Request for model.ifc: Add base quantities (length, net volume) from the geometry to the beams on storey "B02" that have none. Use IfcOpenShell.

First a look at what the model holds.

```python
import ifcopenshell
import ifcopenshell.util.element
import ifcopenshell.util.unit

model = ifcopenshell.open("model.ifc")
print(model.schema)
for unit_type in ("LENGTHUNIT", "AREAUNIT", "VOLUMEUNIT"):
    print(unit_type, ifcopenshell.util.unit.calculate_unit_scale(model, unit_type))
storey = next(s for s in model.by_type("IfcBuildingStorey") if s.Name == "B02")
beams = [e for e in ifcopenshell.util.element.get_decomposition(storey) if e.is_a("IfcBeam")]
for e in sorted(beams, key=lambda e: e.id()):
    print(e.id(), e.is_a(), e.Name, list(ifcopenshell.util.element.get_psets(e, qtos_only=True)), sep=" | ")
```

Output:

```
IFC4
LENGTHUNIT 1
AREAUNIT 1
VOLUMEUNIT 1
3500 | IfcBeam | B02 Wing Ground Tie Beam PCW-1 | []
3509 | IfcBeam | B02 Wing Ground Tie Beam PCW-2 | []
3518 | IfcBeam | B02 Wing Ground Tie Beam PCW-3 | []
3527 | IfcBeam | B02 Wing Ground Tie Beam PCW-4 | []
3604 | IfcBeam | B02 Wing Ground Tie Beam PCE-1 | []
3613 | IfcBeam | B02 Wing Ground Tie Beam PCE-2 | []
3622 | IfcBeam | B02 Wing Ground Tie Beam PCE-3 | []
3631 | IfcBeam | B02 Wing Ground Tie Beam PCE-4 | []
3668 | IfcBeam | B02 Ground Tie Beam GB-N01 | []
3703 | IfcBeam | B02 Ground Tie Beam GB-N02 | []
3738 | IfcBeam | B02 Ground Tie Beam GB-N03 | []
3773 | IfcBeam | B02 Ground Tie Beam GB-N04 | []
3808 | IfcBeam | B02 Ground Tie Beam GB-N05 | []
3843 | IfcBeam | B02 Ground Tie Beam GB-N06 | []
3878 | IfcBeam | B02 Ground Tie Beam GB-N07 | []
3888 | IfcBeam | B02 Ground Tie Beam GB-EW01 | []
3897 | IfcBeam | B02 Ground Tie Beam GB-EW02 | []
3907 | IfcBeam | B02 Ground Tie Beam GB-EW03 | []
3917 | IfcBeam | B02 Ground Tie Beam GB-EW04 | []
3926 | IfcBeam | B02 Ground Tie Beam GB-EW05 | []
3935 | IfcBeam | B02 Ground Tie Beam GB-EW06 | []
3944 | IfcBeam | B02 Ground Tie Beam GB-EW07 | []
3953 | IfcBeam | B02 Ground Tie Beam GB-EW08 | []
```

```python
import ifcopenshell
import ifcopenshell.api.pset
import ifcopenshell.geom
import ifcopenshell.util.element
import ifcopenshell.util.shape
import ifcopenshell.util.unit

model = ifcopenshell.open("model.ifc")
unit_scale = ifcopenshell.util.unit.calculate_unit_scale(model)
volume_scale = ifcopenshell.util.unit.calculate_unit_scale(model, "VOLUMEUNIT")
settings = ifcopenshell.geom.settings()

storey = next(s for s in model.by_type("IfcBuildingStorey") if s.Name == "B02")
beams = [e for e in ifcopenshell.util.element.get_decomposition(storey) if e.is_a("IfcBeam")]

for e in sorted(beams, key=lambda e: e.id()):
    if ifcopenshell.util.element.get_psets(e, qtos_only=True, should_inherit=False):
        continue
    # Geometry comes back in metres, in the element's own axes.
    shape = ifcopenshell.geom.create_shape(settings, e)
    values = {
        "Length": ifcopenshell.util.shape.get_max_xyz(shape.geometry) / unit_scale,
        "NetVolume": ifcopenshell.util.shape.get_volume(shape.geometry) / volume_scale,
    }
    qto = ifcopenshell.api.pset.add_qto(model, product=e, name="Qto_BeamBaseQuantities")
    ifcopenshell.api.pset.edit_qto(model, qto=qto, properties=values)
    print(e.id(), {k: round(v, 3) for k, v in values.items()})

model.write("model_rev.ifc")
```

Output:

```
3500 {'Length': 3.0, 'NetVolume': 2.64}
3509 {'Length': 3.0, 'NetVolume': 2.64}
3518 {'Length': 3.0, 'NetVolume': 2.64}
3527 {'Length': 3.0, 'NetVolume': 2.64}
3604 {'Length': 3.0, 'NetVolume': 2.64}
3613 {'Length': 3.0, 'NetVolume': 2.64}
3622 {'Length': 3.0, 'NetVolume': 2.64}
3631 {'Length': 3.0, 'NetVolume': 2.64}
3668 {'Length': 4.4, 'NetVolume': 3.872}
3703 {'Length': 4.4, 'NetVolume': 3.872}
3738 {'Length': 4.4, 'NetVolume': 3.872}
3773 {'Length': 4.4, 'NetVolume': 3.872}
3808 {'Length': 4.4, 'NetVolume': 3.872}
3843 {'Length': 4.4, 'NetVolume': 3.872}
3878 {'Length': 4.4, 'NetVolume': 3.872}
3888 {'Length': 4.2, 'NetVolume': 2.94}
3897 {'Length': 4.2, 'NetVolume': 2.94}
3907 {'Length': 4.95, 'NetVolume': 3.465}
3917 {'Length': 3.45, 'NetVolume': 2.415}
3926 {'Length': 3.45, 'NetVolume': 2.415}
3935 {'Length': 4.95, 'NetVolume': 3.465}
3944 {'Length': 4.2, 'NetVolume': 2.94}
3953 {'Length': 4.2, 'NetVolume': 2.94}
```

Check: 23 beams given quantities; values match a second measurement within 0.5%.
